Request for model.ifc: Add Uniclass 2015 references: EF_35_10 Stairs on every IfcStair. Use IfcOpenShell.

First a look at what the model holds.

```python
import ifcopenshell

model = ifcopenshell.open("model.ifc")
print(model.schema)
print("classifications:", [c.Name for c in model.by_type("IfcClassification")])
for ifc_class in ("IfcDoor", "IfcRoof", "IfcStair", "IfcWall", "IfcWindow"):
    print(ifc_class, len(model.by_type(ifc_class)))
```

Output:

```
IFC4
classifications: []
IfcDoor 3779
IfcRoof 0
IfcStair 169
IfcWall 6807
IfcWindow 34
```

```python
import ifcopenshell
import ifcopenshell.api.classification

model = ifcopenshell.open("model.ifc")

system = ifcopenshell.api.classification.add_classification(model, classification="Uniclass 2015")

codes = {
    "IfcStair": ("EF_35_10", "Stairs"),
}
for ifc_class, (code, name) in codes.items():
    products = model.by_type(ifc_class)
    ifcopenshell.api.classification.add_reference(
        model, products=products, classification=system, identification=code, name=name
    )
    print(code, len(products))

model.write("model_rev.ifc")
```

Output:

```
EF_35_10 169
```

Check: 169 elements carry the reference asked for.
